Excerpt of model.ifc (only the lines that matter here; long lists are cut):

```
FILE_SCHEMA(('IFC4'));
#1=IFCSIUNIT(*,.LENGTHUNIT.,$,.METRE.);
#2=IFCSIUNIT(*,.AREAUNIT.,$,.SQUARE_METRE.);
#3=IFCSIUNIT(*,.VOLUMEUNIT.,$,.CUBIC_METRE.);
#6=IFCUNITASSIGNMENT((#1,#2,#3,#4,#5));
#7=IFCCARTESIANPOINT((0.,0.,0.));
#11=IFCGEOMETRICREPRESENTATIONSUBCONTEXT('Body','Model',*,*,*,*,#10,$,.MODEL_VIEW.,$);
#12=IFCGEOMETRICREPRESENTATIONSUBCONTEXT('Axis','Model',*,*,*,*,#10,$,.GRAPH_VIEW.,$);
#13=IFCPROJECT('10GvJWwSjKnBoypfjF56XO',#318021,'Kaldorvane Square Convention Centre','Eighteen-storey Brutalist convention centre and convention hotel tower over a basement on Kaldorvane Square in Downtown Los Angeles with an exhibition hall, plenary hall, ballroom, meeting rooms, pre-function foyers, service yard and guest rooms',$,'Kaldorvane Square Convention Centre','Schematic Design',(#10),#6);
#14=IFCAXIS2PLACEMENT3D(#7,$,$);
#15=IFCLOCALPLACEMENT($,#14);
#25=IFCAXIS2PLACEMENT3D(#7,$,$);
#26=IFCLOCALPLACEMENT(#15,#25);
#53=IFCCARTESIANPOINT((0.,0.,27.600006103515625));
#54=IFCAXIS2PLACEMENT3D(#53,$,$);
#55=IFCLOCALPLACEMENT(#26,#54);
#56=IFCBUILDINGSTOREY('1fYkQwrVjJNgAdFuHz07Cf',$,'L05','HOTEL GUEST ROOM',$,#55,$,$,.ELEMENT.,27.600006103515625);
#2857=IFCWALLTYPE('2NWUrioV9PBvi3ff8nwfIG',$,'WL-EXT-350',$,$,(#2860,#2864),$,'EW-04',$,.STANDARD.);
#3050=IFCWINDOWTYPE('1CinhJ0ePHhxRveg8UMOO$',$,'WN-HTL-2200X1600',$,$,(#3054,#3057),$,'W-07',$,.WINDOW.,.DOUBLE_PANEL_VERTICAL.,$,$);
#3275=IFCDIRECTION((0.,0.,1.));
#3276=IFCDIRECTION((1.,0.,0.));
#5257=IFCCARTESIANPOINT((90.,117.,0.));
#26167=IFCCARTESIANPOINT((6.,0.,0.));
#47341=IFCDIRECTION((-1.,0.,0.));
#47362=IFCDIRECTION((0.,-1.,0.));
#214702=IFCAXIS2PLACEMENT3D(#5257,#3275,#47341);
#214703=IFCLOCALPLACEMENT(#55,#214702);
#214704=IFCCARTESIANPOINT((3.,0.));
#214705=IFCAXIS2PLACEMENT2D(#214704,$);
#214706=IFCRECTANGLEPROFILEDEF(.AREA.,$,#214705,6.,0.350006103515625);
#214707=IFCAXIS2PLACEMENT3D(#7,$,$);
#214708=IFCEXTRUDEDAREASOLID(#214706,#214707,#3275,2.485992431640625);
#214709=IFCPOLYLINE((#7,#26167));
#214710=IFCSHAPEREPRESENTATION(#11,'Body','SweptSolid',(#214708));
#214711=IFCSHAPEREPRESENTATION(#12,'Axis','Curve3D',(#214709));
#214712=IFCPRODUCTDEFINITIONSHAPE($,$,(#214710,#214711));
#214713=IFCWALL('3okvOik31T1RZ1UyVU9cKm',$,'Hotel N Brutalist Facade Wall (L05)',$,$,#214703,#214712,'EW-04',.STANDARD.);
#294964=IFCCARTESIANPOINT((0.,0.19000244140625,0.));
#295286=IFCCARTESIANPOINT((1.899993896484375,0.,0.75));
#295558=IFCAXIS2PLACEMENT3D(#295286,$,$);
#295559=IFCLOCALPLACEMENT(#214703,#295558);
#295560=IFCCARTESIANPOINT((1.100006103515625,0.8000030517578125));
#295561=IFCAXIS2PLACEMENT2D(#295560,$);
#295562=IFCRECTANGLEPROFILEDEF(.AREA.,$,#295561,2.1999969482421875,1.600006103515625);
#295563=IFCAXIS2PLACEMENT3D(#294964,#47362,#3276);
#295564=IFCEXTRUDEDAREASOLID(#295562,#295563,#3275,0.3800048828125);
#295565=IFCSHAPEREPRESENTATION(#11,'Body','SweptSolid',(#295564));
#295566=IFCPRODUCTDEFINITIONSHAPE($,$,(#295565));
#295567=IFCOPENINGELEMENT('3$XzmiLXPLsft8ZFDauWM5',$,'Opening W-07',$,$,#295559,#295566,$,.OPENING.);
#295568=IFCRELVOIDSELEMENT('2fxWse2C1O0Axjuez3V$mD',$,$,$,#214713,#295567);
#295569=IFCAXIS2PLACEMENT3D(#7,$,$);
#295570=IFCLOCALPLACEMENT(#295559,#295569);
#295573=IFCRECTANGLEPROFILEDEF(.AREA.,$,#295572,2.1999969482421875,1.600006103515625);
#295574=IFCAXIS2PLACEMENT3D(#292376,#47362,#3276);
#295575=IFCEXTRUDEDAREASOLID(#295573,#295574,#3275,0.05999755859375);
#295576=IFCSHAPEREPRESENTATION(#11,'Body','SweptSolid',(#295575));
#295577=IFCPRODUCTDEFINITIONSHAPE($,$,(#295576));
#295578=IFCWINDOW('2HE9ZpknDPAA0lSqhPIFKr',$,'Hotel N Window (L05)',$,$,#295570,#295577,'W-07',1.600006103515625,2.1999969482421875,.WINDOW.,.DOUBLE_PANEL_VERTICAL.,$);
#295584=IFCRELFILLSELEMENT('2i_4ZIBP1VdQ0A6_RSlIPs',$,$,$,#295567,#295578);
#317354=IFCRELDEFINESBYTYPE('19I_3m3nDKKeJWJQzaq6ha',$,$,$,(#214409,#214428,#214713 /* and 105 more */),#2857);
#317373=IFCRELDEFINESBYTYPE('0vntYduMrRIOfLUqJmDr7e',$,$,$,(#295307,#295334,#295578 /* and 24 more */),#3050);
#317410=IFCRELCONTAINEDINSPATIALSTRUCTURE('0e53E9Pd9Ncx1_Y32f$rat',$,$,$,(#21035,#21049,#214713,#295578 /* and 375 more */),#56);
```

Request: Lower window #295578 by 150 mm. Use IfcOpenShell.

```python
import numpy as np
import ifcopenshell
import ifcopenshell.api.geometry
import ifcopenshell.util.placement
import ifcopenshell.util.unit

model = ifcopenshell.open("model.ifc")
unit_scale = ifcopenshell.util.unit.calculate_unit_scale(model)

window = model.by_guid("2HE9ZpknDPAA0lSqhPIFKr")
opening = window.FillsVoids[0].RelatingOpeningElement
dz = -0.15 / unit_scale

shift = np.array([0.0, 0.0, dz])
# The window is placed relative to its opening, so it follows when the opening moves.
matrix = ifcopenshell.util.placement.get_local_placement(opening.ObjectPlacement)
matrix[:3, 3] += shift
ifcopenshell.api.geometry.edit_object_placement(
    model, product=opening, matrix=matrix, is_si=False, should_transform_children=True
)

print(f"moved by {dz * unit_scale:+.3f} m")

model.write("model_updated.ifc")
```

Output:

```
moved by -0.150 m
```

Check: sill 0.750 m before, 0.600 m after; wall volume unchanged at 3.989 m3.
